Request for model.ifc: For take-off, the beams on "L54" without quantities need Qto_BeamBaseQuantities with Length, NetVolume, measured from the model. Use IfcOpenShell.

First a look at what the model holds.

```python
import ifcopenshell
import ifcopenshell.util.element
import ifcopenshell.util.unit

model = ifcopenshell.open("model.ifc")
print(model.schema)
for unit_type in ("LENGTHUNIT", "AREAUNIT", "VOLUMEUNIT"):
    print(unit_type, ifcopenshell.util.unit.calculate_unit_scale(model, unit_type))
storey = next(s for s in model.by_type("IfcBuildingStorey") if s.Name == "L54")
beams = [e for e in ifcopenshell.util.element.get_decomposition(storey) if e.is_a("IfcBeam")]
for e in sorted(beams, key=lambda e: e.id()):
    print(e.id(), e.is_a(), e.Name, list(ifcopenshell.util.element.get_psets(e, qtos_only=True)), sep=" | ")
```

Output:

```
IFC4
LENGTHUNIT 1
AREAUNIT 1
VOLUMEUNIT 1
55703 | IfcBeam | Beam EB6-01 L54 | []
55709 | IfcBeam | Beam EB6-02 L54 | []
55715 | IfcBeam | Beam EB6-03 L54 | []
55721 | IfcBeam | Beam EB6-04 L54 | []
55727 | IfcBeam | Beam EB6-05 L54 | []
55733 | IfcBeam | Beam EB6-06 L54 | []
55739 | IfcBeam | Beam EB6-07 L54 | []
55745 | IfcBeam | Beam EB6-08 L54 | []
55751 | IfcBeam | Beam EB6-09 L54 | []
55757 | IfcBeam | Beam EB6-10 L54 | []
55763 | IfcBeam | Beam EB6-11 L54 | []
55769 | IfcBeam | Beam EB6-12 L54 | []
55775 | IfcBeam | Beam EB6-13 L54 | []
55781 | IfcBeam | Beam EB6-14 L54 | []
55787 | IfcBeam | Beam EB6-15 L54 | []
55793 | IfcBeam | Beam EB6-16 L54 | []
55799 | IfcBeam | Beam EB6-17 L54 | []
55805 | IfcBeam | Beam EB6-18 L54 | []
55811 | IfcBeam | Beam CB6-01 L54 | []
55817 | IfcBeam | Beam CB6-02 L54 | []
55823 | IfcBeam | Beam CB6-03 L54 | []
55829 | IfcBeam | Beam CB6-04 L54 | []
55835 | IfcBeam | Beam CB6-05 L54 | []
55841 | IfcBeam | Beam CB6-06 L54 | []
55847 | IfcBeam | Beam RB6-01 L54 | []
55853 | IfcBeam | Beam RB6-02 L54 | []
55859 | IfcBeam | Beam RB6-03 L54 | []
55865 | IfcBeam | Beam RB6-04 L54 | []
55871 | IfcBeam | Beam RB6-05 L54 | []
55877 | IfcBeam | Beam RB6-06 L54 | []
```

```python
import ifcopenshell
import ifcopenshell.api.pset
import ifcopenshell.geom
import ifcopenshell.util.element
import ifcopenshell.util.shape
import ifcopenshell.util.unit

model = ifcopenshell.open("model.ifc")
unit_scale = ifcopenshell.util.unit.calculate_unit_scale(model)
volume_scale = ifcopenshell.util.unit.calculate_unit_scale(model, "VOLUMEUNIT")
settings = ifcopenshell.geom.settings()

storey = next(s for s in model.by_type("IfcBuildingStorey") if s.Name == "L54")
beams = [e for e in ifcopenshell.util.element.get_decomposition(storey) if e.is_a("IfcBeam")]

for e in sorted(beams, key=lambda e: e.id()):
    if ifcopenshell.util.element.get_psets(e, qtos_only=True, should_inherit=False):
        continue
    # Geometry comes back in metres, in the element's own axes.
    shape = ifcopenshell.geom.create_shape(settings, e)
    values = {
        "Length": ifcopenshell.util.shape.get_max_xyz(shape.geometry) / unit_scale,
        "NetVolume": ifcopenshell.util.shape.get_volume(shape.geometry) / volume_scale,
    }
    qto = ifcopenshell.api.pset.add_qto(model, product=e, name="Qto_BeamBaseQuantities")
    ifcopenshell.api.pset.edit_qto(model, qto=qto, properties=values)
    print(e.id(), {k: round(v, 3) for k, v in values.items()})

model.write("model_rev.ifc")
```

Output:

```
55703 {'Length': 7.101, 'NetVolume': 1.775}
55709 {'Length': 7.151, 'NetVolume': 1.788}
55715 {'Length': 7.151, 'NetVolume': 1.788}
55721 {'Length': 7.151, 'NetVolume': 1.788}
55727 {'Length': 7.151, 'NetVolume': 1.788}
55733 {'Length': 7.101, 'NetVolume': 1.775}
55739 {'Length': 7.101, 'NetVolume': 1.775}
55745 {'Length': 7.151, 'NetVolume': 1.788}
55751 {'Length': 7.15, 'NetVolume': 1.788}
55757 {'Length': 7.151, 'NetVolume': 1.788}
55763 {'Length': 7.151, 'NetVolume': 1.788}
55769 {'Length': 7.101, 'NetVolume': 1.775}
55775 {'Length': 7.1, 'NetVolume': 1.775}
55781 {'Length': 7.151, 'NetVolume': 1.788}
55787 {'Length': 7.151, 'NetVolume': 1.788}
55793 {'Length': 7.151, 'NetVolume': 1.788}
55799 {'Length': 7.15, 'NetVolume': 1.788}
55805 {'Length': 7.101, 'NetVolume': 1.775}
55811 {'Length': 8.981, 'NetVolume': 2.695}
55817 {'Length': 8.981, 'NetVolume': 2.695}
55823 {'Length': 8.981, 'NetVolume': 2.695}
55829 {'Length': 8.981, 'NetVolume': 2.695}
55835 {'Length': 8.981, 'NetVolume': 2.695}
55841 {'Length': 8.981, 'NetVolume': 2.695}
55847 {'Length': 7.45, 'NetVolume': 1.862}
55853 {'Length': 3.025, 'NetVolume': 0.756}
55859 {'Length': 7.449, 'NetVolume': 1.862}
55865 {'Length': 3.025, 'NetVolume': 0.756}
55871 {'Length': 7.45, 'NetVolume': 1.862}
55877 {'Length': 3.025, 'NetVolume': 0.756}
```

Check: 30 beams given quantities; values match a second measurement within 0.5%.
